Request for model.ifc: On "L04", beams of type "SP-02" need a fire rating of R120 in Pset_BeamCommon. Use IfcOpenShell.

First a look at what the model holds.

```python
import ifcopenshell
import ifcopenshell.util.element

model = ifcopenshell.open("model.ifc")
print(model.schema)
storey = next(s for s in model.by_type("IfcBuildingStorey") if s.Name == "L04")
beams = [e for e in ifcopenshell.util.element.get_decomposition(storey) if e.is_a("IfcBeam")]
seen = {}
for e in beams:
    element_type = ifcopenshell.util.element.get_type(e)
    key = (element_type.Name if element_type != e and element_type else None, ifcopenshell.util.element.get_pset(e, "Pset_BeamCommon", "FireRating"))
    seen[key] = seen.get(key, 0) + 1
for (name, value), count in sorted(seen.items(), key=str):
    print(count, "x", name, "|", value)
```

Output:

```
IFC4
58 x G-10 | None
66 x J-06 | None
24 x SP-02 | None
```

```python
import ifcopenshell
import ifcopenshell.api.pset
import ifcopenshell.util.element

model = ifcopenshell.open("model.ifc")

storey = next(s for s in model.by_type("IfcBuildingStorey") if s.Name == "L04")
beams = [e for e in ifcopenshell.util.element.get_decomposition(storey) if e.is_a("IfcBeam")]

count = 0
for e in beams:
    element_type = ifcopenshell.util.element.get_type(e)
    if element_type in (None, e) or element_type.Name != "SP-02":
        continue
    # add_pset returns the element's existing set when there is one.
    pset = ifcopenshell.api.pset.add_pset(model, product=e, name="Pset_BeamCommon")
    ifcopenshell.api.pset.edit_pset(model, pset=pset, properties={"FireRating": "R120"})
    count += 1

print(count, "beams updated")

model.write("model_rev.ifc")
```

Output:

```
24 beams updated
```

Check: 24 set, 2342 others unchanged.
